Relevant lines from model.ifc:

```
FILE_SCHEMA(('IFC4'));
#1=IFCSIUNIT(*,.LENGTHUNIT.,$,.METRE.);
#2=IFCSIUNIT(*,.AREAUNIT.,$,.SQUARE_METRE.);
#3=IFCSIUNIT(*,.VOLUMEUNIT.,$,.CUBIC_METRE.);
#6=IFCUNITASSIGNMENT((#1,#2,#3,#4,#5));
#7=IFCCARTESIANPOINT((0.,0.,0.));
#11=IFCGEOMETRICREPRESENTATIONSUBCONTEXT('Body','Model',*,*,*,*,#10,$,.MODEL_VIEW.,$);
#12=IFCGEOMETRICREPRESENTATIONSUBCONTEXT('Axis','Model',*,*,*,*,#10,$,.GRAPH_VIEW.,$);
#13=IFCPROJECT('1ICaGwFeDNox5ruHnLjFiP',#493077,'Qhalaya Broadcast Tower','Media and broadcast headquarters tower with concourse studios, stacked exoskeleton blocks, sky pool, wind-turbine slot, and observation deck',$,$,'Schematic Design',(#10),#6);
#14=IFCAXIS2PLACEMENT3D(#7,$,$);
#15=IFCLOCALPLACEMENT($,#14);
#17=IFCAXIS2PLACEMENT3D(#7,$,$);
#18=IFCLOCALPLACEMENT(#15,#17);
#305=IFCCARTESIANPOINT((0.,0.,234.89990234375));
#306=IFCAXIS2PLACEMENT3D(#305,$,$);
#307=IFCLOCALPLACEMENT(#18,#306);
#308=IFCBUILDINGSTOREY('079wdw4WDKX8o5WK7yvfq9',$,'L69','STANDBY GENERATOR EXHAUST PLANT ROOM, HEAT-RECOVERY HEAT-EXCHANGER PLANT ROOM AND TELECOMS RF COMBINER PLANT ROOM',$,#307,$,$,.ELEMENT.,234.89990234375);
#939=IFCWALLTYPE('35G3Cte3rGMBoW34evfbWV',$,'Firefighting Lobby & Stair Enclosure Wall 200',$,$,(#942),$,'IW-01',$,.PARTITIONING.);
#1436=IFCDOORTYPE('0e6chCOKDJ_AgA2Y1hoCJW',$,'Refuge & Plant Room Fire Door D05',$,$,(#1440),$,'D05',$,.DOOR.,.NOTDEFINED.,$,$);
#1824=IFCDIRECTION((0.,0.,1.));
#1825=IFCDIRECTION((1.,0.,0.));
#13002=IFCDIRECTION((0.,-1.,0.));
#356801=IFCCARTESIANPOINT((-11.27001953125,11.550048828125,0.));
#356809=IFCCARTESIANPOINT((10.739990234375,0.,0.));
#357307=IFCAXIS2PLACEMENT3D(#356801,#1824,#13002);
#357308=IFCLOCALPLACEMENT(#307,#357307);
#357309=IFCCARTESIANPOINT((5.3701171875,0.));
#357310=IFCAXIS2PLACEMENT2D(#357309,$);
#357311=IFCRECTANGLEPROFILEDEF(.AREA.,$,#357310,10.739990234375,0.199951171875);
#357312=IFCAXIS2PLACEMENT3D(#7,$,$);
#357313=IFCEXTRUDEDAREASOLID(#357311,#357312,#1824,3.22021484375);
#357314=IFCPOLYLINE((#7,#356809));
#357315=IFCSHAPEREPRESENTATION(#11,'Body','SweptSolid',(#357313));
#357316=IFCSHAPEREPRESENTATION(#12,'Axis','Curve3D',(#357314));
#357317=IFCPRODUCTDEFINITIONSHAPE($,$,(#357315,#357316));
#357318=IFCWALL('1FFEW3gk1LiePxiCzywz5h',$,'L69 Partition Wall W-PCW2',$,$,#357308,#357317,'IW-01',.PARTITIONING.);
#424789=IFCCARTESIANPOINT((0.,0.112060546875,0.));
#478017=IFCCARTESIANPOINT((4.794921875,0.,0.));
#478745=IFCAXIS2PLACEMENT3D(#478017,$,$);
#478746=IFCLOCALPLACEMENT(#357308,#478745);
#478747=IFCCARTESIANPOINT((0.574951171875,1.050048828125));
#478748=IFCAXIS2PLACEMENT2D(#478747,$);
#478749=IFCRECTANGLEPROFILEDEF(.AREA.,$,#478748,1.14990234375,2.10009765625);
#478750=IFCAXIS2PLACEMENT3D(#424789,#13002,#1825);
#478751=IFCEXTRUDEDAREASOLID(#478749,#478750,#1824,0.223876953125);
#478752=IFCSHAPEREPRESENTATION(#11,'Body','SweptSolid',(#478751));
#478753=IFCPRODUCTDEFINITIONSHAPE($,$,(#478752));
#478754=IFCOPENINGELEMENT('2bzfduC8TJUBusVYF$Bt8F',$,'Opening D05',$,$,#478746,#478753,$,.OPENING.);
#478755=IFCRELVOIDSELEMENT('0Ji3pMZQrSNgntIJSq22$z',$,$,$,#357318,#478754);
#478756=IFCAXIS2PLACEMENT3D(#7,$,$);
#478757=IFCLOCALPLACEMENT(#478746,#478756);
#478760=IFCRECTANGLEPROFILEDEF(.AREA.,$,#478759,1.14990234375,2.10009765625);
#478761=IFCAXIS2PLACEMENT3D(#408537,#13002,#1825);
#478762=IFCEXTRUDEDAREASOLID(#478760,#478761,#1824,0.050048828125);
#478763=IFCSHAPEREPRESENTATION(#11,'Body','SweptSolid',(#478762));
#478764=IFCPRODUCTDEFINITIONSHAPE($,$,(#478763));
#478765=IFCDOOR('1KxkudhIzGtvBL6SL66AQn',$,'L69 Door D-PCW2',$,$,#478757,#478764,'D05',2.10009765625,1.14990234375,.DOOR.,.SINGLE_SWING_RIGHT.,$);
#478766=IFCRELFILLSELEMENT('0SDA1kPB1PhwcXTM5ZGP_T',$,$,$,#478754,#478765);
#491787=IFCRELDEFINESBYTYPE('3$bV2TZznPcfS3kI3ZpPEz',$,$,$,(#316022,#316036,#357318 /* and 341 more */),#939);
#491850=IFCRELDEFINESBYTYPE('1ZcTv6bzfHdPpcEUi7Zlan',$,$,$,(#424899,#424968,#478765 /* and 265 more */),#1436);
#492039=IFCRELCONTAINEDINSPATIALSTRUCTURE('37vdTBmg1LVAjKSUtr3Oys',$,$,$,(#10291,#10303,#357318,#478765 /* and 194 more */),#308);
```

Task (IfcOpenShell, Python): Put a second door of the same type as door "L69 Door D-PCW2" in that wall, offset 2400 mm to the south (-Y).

```python
import ifcopenshell
import ifcopenshell.api.feature
import ifcopenshell.api.geometry
import ifcopenshell.api.root
import ifcopenshell.geom
import ifcopenshell.util.element
import ifcopenshell.util.placement
import ifcopenshell.util.shape

model = ifcopenshell.open("model.ifc")
settings = ifcopenshell.geom.settings()


def volume(element):
    """Net volume in cubic metres, openings subtracted."""
    shape = ifcopenshell.geom.create_shape(settings, element)
    return ifcopenshell.util.shape.get_volume(shape.geometry)


door = model.by_guid("1KxkudhIzGtvBL6SL66AQn")
opening = door.FillsVoids[0].RelatingOpeningElement
wall = opening.VoidsElements[0].RelatingBuildingElement
before = volume(wall)
shift = ifcopenshell.util.placement.get_local_placement(wall.ObjectPlacement)[:3, 0] * 2.4

# copy_class copies the void relationship, type, container and properties, but no geometry.
new_opening = ifcopenshell.api.root.copy_class(model, product=opening)
new_opening.Representation = ifcopenshell.util.element.copy_deep(
    model, opening.Representation, exclude=["IfcGeometricRepresentationContext", "IfcRepresentationMap"]
)
new_door = ifcopenshell.api.root.copy_class(model, product=door)
new_door.Representation = ifcopenshell.util.element.copy_deep(
    model, door.Representation, exclude=["IfcGeometricRepresentationContext", "IfcRepresentationMap"]
)
new_door.Tag = None
ifcopenshell.api.feature.add_filling(model, opening=new_opening, element=new_door)

for old, new in ((opening, new_opening), (door, new_door)):
    matrix = ifcopenshell.util.placement.get_local_placement(old.ObjectPlacement)
    matrix[:3, 3] += shift
    ifcopenshell.api.geometry.edit_object_placement(model, product=new, matrix=matrix, is_si=False)

after = volume(wall)

print(f"wall volume {before:.3f} -> {after:.3f} m3")

model.write("model_edited.ifc")
```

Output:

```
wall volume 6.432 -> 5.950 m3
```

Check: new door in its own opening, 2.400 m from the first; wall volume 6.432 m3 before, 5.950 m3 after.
